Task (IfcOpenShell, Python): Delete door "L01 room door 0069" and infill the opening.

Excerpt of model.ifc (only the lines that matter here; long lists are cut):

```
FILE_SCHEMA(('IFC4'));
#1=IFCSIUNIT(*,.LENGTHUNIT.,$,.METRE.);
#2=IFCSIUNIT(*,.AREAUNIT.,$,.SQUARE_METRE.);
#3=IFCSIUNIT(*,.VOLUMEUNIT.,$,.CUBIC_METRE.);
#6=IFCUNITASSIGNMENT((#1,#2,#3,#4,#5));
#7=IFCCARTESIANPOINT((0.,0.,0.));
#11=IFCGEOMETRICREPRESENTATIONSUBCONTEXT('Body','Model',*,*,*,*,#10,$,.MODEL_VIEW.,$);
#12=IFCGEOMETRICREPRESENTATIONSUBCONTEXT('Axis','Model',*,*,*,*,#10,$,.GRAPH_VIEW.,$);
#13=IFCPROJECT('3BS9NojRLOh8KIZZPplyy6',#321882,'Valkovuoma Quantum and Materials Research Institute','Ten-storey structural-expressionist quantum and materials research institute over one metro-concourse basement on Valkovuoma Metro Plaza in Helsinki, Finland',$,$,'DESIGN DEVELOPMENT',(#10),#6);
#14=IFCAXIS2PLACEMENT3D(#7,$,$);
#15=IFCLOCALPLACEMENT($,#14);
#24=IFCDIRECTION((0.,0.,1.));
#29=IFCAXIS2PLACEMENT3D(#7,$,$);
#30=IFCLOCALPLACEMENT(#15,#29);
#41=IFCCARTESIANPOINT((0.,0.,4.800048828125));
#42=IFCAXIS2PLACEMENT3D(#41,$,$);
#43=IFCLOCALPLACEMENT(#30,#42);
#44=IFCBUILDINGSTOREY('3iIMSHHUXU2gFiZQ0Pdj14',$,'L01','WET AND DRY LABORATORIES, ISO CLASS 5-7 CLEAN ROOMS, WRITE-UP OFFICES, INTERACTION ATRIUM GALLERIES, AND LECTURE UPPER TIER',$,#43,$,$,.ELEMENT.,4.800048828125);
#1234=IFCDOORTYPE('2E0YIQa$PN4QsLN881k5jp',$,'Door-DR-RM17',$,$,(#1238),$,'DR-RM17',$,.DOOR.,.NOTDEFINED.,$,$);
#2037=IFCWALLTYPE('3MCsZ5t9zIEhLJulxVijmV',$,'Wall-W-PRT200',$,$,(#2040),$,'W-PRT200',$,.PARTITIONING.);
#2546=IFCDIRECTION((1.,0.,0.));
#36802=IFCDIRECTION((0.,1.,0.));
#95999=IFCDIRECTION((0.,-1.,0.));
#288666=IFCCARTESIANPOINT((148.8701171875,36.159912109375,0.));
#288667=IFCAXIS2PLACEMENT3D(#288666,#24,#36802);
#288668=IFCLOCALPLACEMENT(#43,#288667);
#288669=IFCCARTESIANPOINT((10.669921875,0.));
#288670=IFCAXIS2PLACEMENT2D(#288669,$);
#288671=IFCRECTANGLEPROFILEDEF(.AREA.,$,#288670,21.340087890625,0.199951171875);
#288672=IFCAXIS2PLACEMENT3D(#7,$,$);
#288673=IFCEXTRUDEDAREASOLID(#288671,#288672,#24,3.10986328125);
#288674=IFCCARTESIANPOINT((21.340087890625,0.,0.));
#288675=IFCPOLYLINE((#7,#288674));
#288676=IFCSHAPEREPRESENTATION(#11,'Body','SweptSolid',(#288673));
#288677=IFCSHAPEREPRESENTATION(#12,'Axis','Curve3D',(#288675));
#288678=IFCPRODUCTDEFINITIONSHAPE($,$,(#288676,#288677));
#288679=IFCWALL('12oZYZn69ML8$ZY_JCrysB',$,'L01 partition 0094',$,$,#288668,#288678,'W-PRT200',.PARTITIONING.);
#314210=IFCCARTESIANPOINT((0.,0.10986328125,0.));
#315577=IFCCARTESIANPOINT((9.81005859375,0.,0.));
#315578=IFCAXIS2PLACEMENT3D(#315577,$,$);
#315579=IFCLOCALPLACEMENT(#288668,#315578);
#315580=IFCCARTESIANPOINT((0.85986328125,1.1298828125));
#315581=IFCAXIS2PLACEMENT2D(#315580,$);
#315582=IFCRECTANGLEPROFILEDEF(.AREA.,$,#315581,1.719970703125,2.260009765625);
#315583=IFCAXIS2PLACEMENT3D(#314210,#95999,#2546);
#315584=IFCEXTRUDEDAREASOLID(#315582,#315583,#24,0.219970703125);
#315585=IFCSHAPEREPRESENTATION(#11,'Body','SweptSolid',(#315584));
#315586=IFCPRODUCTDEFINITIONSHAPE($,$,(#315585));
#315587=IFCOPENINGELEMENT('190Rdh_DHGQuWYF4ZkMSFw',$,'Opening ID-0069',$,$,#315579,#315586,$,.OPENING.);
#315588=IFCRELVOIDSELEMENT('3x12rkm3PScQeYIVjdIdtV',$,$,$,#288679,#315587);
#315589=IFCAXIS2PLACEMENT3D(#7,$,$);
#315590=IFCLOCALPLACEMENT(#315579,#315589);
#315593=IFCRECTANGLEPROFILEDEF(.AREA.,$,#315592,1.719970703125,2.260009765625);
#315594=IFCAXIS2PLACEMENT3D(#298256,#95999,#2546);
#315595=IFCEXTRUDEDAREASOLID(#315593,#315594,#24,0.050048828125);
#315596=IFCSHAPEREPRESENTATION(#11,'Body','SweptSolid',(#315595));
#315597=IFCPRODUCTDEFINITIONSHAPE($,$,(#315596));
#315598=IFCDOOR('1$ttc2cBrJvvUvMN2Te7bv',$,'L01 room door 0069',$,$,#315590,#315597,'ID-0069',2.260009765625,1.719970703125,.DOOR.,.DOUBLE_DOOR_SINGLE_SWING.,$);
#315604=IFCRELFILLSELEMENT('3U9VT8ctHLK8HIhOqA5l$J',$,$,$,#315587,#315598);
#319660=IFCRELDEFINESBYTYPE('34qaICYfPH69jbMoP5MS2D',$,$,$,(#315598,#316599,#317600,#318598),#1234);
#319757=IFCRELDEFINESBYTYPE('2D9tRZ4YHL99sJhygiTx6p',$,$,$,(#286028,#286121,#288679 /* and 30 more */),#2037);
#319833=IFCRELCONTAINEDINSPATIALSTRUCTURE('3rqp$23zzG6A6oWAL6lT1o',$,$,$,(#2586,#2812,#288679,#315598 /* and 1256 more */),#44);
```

```python
import ifcopenshell
import ifcopenshell.api.feature
import ifcopenshell.api.root
import ifcopenshell.geom
import ifcopenshell.util.shape

model = ifcopenshell.open("model.ifc")
settings = ifcopenshell.geom.settings()


def volume(element):
    """Net volume in cubic metres, openings subtracted."""
    shape = ifcopenshell.geom.create_shape(settings, element)
    return ifcopenshell.util.shape.get_volume(shape.geometry)


door = model.by_id(315598)
opening = door.FillsVoids[0].RelatingOpeningElement
wall = opening.VoidsElements[0].RelatingBuildingElement
before = volume(wall)

ifcopenshell.api.root.remove_product(model, product=door)
ifcopenshell.api.feature.remove_feature(model, feature=opening)

after = volume(wall)

print(f"wall volume {before:.3f} -> {after:.3f} m3")

model.write("model-out.ifc")
```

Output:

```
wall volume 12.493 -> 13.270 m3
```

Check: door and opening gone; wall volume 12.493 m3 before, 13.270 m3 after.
